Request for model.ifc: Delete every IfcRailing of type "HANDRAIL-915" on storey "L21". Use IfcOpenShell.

First a look at what the model holds.

```python
import ifcopenshell
import ifcopenshell.util.element

model = ifcopenshell.open("model.ifc")
print(model.schema)
storey = next(s for s in model.by_type("IfcBuildingStorey") if s.Name == "L21")
railings = [e for e in ifcopenshell.util.element.get_decomposition(storey) if e.is_a("IfcRailing")]
seen = {}
for e in railings:
    element_type = ifcopenshell.util.element.get_type(e)
    name = element_type.Name if element_type not in (None, e) else None
    seen[name] = seen.get(name, 0) + 1
for name, count in sorted(seen.items(), key=str):
    print(count, "x", name)
```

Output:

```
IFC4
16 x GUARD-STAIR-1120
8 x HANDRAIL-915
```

```python
import ifcopenshell
import ifcopenshell.api.root
import ifcopenshell.util.element

model = ifcopenshell.open("model.ifc")

storey = next(s for s in model.by_type("IfcBuildingStorey") if s.Name == "L21")
railings = [e for e in ifcopenshell.util.element.get_decomposition(storey) if e.is_a("IfcRailing")]
targets = [e for e in railings if (t := ifcopenshell.util.element.get_type(e)) not in (None, e) and t.Name == "HANDRAIL-915"]

for e in targets:
    ifcopenshell.api.root.remove_product(model, product=e)
print(len(targets), "removed")

model.write("model_rev.ifc")
```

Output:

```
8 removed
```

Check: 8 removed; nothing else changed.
